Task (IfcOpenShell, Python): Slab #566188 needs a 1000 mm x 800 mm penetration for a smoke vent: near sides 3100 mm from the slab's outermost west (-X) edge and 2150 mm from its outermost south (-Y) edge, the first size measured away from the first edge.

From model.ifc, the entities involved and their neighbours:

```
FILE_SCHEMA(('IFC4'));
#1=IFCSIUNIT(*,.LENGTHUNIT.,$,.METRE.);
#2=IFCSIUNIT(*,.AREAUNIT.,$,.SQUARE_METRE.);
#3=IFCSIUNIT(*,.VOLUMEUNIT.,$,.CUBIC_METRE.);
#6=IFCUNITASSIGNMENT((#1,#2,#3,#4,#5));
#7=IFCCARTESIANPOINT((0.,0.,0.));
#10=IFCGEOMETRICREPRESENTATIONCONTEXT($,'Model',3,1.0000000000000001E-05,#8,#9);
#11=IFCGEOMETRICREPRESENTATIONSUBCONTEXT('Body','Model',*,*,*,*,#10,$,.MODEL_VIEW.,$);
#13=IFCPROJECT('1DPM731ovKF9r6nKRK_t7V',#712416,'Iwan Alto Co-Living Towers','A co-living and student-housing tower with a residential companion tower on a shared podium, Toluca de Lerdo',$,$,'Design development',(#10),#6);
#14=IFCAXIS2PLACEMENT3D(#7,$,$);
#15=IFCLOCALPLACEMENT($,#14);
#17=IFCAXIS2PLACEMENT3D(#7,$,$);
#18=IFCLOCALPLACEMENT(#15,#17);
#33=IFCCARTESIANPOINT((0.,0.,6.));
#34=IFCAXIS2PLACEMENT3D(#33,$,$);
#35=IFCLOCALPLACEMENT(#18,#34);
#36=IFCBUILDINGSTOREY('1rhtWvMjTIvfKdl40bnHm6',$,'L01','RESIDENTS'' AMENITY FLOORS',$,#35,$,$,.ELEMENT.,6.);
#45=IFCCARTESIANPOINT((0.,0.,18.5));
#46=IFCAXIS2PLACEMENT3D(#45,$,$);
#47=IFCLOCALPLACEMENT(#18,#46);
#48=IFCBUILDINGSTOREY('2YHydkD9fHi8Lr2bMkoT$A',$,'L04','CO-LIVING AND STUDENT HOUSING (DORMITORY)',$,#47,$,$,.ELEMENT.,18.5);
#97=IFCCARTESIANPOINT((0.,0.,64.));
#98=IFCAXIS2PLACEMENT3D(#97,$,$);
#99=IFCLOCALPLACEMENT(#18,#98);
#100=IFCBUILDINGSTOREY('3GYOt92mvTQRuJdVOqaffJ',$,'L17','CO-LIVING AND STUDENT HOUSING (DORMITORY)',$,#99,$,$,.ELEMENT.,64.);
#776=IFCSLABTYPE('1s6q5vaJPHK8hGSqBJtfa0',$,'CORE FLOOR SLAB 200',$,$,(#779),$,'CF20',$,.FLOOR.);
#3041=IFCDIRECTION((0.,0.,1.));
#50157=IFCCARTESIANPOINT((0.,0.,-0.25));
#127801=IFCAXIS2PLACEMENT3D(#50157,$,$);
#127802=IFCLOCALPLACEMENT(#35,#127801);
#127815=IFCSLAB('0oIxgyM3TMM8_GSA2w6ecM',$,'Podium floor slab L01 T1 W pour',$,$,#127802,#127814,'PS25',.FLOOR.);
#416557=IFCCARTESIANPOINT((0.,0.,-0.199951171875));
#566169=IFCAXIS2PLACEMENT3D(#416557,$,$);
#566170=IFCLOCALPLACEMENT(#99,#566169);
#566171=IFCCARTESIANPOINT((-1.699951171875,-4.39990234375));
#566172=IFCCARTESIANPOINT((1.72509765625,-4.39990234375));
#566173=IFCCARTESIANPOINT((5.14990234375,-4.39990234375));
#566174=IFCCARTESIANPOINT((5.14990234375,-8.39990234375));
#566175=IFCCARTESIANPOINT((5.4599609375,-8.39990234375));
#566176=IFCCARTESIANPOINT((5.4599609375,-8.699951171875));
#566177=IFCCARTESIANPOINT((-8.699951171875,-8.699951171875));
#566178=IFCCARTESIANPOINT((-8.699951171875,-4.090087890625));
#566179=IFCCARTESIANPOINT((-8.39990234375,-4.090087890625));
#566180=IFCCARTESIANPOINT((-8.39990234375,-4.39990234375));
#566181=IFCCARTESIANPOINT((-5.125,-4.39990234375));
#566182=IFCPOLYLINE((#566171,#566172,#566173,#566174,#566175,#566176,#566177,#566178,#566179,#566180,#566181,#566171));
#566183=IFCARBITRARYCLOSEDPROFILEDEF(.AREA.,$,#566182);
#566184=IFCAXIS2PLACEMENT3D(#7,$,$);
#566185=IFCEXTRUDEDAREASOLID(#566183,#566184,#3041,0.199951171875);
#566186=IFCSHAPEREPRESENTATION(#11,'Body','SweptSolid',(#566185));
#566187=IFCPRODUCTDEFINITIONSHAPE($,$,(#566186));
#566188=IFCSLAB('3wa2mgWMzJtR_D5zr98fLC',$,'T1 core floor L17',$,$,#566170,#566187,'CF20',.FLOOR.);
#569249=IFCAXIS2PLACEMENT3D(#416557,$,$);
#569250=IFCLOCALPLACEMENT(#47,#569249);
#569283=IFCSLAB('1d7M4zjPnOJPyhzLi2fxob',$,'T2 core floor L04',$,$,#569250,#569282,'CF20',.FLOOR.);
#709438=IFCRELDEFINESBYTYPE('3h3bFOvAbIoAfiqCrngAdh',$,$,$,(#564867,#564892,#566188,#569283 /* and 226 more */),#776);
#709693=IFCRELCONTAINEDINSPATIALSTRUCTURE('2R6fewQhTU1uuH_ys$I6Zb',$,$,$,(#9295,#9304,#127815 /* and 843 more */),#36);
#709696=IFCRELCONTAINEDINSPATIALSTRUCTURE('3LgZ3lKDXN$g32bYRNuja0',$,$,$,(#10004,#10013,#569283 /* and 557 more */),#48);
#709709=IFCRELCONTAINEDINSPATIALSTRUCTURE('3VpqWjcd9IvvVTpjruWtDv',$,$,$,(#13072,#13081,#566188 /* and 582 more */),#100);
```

```python
import numpy as np
import ifcopenshell
import ifcopenshell.api.feature
import ifcopenshell.api.geometry
import ifcopenshell.api.root
import ifcopenshell.geom
import ifcopenshell.util.placement
import ifcopenshell.util.representation
import ifcopenshell.util.shape
import ifcopenshell.util.unit

model = ifcopenshell.open("model.ifc")
unit_scale = ifcopenshell.util.unit.calculate_unit_scale(model)
settings = ifcopenshell.geom.settings()


def volume(element):
    """Net volume in cubic metres, openings subtracted."""
    shape = ifcopenshell.geom.create_shape(settings, element)
    return ifcopenshell.util.shape.get_volume(shape.geometry)


slab = model.by_guid("3wa2mgWMzJtR_D5zr98fLC")
before = volume(slab)

# Extent in the slab's own axes, in metres. The edges named are its -X and -Y sides.
slab_shape = ifcopenshell.geom.create_shape(settings, slab)
vertices = ifcopenshell.util.shape.get_vertices(slab_shape.geometry)
x_min, y_min, bottom = vertices.min(axis=0)
top = vertices[:, 2].max()

opening = ifcopenshell.api.root.create_entity(model, ifc_class="IfcOpeningElement", name="Smoke vent opening", predefined_type="OPENING")
context = ifcopenshell.util.representation.get_context(model, "Model", "Body", "MODEL_VIEW")
width, depth = 1, 0.8
outline = [(0.0, 0.0), (width, 0.0), (width, depth), (0.0, depth), (0.0, 0.0)]
# Overshoot both faces by 50 mm so the cut is clean.
shape = ifcopenshell.api.geometry.add_slab_representation(
    model, context=context, depth=top - bottom + 0.1, polyline=outline
)
ifcopenshell.api.geometry.assign_representation(model, product=opening, representation=shape)

matrix = ifcopenshell.util.placement.get_local_placement(slab.ObjectPlacement)
matrix[:, 3] = matrix @ np.append(np.array([x_min + 3.1, y_min + 2.15, bottom - 0.05]) / unit_scale, 1.0)
ifcopenshell.api.geometry.edit_object_placement(model, product=opening, matrix=matrix, is_si=False)
ifcopenshell.api.feature.add_feature(model, feature=opening, element=slab)

after = volume(slab)

print(f"slab volume {before:.3f} -> {after:.3f} m3")

model.write("model_updated.ifc")
```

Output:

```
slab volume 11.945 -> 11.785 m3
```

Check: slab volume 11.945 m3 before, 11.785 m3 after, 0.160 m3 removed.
